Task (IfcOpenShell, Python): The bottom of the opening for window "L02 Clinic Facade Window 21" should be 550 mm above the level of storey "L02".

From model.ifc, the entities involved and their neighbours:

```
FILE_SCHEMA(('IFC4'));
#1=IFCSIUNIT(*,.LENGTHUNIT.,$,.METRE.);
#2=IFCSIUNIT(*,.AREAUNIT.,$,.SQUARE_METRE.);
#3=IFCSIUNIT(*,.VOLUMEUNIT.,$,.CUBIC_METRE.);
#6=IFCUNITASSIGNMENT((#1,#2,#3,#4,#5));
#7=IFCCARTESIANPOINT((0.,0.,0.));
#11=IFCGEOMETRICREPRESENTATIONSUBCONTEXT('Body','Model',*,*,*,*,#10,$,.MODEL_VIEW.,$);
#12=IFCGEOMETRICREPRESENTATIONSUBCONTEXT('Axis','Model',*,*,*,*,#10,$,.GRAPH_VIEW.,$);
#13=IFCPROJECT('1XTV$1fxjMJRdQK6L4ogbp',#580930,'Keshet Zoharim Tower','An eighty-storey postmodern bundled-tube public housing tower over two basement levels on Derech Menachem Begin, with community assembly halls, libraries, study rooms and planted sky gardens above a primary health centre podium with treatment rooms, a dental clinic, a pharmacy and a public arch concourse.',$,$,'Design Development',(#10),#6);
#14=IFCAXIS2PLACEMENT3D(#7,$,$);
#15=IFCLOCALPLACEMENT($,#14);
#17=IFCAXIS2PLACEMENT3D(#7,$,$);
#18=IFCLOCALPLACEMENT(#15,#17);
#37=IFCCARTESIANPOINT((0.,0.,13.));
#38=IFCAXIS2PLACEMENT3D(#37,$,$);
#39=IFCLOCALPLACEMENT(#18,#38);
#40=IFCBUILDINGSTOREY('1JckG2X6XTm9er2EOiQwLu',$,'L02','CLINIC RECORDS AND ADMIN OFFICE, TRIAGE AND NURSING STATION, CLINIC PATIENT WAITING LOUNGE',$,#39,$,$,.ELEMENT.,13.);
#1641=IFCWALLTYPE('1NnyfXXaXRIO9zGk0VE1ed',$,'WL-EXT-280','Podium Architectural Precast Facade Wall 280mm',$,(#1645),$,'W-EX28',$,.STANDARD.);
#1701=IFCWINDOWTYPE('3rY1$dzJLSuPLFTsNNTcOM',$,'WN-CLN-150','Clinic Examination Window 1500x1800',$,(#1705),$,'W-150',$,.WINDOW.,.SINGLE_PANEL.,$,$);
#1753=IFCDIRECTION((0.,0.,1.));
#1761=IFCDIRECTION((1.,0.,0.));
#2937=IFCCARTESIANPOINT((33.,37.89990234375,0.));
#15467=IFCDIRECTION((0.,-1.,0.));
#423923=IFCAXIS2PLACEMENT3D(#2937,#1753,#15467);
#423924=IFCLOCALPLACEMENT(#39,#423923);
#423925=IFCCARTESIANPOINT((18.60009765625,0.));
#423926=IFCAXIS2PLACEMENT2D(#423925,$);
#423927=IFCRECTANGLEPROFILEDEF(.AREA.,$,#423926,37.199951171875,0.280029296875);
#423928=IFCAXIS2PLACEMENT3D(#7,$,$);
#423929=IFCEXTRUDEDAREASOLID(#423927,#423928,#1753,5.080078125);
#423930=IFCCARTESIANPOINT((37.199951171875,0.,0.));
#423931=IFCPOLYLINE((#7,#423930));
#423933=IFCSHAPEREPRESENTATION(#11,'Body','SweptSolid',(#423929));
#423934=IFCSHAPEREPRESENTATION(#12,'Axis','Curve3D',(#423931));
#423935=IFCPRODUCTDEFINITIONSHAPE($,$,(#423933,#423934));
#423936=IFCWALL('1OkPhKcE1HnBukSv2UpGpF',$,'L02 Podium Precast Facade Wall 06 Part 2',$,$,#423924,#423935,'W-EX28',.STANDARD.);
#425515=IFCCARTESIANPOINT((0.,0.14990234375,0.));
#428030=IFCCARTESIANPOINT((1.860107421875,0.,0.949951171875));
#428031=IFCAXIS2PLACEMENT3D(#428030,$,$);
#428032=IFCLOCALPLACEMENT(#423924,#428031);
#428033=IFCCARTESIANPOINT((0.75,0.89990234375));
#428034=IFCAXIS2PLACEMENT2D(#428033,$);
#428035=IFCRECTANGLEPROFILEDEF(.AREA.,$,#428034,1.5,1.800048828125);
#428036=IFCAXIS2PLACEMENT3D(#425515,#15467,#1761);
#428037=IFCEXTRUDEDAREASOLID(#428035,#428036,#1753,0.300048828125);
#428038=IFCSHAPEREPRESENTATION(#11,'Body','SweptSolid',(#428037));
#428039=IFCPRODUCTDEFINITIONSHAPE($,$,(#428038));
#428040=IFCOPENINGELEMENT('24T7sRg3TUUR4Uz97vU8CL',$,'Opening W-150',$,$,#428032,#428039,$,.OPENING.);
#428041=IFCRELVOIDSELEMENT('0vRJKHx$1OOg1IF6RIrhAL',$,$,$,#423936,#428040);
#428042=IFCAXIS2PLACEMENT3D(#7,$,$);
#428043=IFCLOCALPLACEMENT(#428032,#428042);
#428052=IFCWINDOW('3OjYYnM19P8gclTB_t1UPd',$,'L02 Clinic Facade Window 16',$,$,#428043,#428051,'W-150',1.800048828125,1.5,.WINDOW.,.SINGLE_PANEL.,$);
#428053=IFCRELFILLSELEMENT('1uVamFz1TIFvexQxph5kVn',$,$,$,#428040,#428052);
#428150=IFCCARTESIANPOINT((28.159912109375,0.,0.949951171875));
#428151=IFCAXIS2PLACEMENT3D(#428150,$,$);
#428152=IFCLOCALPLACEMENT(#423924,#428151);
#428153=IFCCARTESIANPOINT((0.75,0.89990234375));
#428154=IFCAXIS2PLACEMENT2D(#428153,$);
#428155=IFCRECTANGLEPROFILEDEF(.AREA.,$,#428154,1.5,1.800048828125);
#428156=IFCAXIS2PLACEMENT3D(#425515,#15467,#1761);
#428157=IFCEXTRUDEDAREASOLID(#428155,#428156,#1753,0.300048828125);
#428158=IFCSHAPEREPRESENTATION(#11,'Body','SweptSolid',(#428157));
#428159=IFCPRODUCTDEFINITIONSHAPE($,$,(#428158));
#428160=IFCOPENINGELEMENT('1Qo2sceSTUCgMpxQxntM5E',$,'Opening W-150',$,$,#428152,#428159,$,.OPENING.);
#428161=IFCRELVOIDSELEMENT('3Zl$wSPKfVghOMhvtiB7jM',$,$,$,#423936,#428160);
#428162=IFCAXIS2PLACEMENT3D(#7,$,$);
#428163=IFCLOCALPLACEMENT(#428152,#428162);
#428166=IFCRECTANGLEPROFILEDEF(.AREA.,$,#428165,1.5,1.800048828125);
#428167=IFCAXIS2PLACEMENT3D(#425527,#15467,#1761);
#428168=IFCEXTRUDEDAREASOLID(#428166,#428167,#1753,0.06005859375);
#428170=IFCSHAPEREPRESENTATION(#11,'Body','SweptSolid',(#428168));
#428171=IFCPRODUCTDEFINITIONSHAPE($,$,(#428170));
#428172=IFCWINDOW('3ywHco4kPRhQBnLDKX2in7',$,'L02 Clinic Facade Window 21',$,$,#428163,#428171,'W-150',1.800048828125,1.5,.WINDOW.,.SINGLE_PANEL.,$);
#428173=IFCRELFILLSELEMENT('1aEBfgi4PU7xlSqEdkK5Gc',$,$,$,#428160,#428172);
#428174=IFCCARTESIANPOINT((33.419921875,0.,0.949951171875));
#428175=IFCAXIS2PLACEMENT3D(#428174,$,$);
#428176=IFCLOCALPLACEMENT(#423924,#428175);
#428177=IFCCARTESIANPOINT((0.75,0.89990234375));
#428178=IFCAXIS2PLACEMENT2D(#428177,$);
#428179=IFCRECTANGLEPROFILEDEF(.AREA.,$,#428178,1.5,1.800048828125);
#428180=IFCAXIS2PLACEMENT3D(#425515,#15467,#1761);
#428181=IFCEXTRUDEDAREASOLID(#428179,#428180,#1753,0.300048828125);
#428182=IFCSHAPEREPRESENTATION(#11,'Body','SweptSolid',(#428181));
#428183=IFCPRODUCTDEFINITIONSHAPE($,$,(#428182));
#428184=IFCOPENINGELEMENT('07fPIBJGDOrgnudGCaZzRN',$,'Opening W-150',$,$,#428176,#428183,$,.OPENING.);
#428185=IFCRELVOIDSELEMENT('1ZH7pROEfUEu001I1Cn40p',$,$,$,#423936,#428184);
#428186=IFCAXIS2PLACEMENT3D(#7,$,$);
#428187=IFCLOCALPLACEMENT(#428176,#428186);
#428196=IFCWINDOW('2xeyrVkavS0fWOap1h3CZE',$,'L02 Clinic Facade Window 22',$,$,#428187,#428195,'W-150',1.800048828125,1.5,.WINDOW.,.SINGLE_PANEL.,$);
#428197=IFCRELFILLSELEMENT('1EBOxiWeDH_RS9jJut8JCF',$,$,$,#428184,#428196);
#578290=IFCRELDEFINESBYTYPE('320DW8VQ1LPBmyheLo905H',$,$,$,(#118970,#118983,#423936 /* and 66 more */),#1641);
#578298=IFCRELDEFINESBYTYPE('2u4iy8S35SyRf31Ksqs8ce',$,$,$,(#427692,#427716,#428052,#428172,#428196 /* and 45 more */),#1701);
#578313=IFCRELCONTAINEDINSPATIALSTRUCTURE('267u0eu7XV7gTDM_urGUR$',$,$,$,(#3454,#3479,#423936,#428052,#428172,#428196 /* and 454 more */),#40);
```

```python
import numpy as np
import ifcopenshell
import ifcopenshell.api.geometry
import ifcopenshell.geom
import ifcopenshell.util.element
import ifcopenshell.util.placement
import ifcopenshell.util.shape
import ifcopenshell.util.unit

model = ifcopenshell.open("model.ifc")
unit_scale = ifcopenshell.util.unit.calculate_unit_scale(model)

window = model.by_id(428172)
opening = window.FillsVoids[0].RelatingOpeningElement
storey = ifcopenshell.util.element.get_container(window, ifc_class="IfcBuildingStorey")
level = ifcopenshell.util.placement.get_local_placement(storey.ObjectPlacement)[2, 3]

# The opening's origin need not be at the sill, so measure its lowest point.
shape = ifcopenshell.geom.create_shape(ifcopenshell.geom.settings(), opening)
bottom = ifcopenshell.util.shape.get_shape_bottom_elevation(shape, shape.geometry) / unit_scale
dz = level + 0.55 - bottom

shift = np.array([0.0, 0.0, dz])
# The window is placed relative to its opening, so it follows when the opening moves.
matrix = ifcopenshell.util.placement.get_local_placement(opening.ObjectPlacement)
matrix[:3, 3] += shift
ifcopenshell.api.geometry.edit_object_placement(
    model, product=opening, matrix=matrix, is_si=False, should_transform_children=True
)

print(f"moved by {dz * unit_scale:+.3f} m")

model.write("model_edited.ifc")
```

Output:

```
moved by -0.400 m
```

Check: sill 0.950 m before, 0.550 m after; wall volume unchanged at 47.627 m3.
